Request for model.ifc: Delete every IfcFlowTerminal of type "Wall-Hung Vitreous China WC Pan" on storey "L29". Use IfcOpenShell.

First a look at what the model holds.

```python
import ifcopenshell
import ifcopenshell.util.element

model = ifcopenshell.open("model.ifc")
print(model.schema)
storey = next(s for s in model.by_type("IfcBuildingStorey") if s.Name == "L29")
terminals = [e for e in ifcopenshell.util.element.get_decomposition(storey) if e.is_a("IfcFlowTerminal")]
seen = {}
for e in terminals:
    element_type = ifcopenshell.util.element.get_type(e)
    name = element_type.Name if element_type not in (None, e) else None
    seen[name] = seen.get(name, 0) + 1
for name, count in sorted(seen.items(), key=str):
    print(count, "x", name)
```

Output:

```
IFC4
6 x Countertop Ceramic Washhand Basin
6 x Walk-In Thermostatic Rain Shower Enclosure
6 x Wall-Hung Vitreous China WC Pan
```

```python
import ifcopenshell
import ifcopenshell.api.root
import ifcopenshell.util.element

model = ifcopenshell.open("model.ifc")

storey = next(s for s in model.by_type("IfcBuildingStorey") if s.Name == "L29")
terminals = [e for e in ifcopenshell.util.element.get_decomposition(storey) if e.is_a("IfcFlowTerminal")]
targets = [e for e in terminals if (t := ifcopenshell.util.element.get_type(e)) not in (None, e) and t.Name == "Wall-Hung Vitreous China WC Pan"]

for e in targets:
    ifcopenshell.api.root.remove_product(model, product=e)
print(len(targets), "removed")

model.write("model-out.ifc")
```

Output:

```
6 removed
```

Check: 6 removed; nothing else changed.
